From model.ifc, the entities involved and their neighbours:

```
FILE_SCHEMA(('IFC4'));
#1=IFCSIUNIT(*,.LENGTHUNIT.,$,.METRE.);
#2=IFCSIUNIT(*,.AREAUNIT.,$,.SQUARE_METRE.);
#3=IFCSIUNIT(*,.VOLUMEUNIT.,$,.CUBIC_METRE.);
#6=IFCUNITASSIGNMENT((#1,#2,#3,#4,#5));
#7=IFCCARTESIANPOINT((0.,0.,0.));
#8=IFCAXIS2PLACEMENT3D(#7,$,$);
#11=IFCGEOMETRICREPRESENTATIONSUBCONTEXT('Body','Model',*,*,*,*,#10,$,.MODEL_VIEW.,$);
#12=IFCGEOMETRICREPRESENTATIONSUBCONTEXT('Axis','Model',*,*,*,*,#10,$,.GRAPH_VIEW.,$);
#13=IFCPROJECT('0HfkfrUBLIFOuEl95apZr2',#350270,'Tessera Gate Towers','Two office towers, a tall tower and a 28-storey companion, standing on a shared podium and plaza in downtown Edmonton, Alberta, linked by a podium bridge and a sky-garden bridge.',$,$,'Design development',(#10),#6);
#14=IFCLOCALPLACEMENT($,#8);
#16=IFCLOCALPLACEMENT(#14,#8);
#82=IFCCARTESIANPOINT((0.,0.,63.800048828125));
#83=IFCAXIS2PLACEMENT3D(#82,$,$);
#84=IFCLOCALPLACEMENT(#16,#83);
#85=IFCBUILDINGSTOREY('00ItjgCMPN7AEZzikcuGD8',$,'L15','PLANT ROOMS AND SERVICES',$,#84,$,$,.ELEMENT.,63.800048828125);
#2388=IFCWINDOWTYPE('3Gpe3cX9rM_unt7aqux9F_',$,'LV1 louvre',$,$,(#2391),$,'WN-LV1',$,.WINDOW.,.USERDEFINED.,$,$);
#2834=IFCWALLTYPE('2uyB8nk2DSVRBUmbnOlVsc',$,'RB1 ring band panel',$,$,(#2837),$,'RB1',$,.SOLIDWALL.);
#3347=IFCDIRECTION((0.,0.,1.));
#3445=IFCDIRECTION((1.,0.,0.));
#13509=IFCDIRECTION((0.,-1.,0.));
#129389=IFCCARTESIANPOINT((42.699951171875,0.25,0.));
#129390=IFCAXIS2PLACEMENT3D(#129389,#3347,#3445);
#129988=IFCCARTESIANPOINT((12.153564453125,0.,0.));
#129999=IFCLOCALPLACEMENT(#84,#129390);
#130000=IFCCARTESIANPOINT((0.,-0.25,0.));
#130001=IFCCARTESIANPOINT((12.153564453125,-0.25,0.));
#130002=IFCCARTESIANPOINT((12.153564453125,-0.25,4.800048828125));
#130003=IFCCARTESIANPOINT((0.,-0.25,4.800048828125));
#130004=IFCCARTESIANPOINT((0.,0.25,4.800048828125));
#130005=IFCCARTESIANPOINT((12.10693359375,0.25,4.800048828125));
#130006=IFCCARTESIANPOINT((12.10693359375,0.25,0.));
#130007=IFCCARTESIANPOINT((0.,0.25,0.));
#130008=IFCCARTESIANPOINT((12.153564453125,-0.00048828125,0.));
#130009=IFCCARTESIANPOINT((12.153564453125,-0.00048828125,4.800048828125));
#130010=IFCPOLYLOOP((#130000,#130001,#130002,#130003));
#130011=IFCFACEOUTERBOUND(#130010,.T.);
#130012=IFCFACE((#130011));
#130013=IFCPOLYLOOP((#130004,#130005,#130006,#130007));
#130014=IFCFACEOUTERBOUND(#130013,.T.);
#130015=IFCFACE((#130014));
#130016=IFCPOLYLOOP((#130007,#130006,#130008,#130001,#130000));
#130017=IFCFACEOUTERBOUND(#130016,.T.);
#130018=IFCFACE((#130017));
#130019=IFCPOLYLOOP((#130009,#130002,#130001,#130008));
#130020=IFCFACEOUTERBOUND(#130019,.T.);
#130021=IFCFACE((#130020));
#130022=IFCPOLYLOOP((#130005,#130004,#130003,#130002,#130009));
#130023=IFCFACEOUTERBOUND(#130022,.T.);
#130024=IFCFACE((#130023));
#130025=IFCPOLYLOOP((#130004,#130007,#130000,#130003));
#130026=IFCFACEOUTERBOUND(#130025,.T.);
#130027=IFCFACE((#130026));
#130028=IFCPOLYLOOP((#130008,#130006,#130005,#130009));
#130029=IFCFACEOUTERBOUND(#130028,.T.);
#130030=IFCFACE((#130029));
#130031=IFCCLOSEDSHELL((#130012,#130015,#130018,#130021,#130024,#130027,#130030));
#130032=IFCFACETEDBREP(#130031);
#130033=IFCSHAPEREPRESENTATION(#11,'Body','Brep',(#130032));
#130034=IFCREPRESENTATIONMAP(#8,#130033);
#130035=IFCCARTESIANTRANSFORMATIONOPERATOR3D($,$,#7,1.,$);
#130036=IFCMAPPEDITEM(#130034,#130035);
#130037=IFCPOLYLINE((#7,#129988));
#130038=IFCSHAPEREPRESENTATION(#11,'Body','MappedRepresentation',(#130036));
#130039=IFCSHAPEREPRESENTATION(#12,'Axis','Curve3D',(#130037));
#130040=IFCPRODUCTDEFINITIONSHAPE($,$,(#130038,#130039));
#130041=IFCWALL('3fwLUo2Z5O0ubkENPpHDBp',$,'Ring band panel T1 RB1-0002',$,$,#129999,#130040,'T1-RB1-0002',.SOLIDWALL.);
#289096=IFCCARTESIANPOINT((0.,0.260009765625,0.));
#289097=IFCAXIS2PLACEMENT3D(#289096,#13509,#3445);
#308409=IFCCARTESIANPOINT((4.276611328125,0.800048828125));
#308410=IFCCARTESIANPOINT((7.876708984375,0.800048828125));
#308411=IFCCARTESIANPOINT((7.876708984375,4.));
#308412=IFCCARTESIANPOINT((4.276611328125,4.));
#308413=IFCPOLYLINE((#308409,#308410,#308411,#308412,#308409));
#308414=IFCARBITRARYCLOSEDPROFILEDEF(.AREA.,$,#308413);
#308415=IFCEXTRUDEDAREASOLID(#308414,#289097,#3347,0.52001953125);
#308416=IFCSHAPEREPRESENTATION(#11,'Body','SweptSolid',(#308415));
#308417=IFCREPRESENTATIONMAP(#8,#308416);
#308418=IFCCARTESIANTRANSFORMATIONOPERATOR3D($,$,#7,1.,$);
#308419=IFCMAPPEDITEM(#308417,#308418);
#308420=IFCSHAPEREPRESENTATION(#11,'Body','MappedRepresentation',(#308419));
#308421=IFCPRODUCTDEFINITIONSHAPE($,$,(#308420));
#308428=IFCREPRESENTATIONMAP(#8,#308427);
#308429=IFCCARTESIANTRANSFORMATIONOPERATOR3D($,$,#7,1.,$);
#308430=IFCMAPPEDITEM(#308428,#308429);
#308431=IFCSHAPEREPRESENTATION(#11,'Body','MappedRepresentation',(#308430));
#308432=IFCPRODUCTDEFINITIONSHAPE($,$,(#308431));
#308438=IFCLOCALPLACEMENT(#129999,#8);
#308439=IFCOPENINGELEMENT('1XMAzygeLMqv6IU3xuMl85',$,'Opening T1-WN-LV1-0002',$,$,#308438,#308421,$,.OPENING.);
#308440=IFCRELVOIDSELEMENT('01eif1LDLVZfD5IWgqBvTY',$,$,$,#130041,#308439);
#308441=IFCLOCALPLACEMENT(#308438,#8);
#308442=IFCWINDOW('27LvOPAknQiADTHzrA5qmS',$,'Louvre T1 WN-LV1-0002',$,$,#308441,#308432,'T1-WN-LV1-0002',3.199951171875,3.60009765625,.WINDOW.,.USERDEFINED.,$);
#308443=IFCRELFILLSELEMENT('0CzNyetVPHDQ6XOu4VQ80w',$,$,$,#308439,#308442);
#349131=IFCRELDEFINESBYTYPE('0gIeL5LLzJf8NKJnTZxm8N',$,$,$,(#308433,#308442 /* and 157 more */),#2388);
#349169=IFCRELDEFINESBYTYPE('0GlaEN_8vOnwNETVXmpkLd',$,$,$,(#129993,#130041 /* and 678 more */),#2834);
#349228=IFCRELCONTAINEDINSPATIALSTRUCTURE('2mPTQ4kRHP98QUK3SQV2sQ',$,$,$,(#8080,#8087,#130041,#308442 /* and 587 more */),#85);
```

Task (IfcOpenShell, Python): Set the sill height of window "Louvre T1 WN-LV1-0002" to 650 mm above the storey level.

```python
import numpy as np
import ifcopenshell
import ifcopenshell.api.geometry
import ifcopenshell.geom
import ifcopenshell.util.element
import ifcopenshell.util.placement
import ifcopenshell.util.shape
import ifcopenshell.util.unit

model = ifcopenshell.open("model.ifc")
unit_scale = ifcopenshell.util.unit.calculate_unit_scale(model)

window = model.by_guid("27LvOPAknQiADTHzrA5qmS")
opening = window.FillsVoids[0].RelatingOpeningElement
storey = ifcopenshell.util.element.get_container(window, ifc_class="IfcBuildingStorey")
level = ifcopenshell.util.placement.get_local_placement(storey.ObjectPlacement)[2, 3]

# The opening's origin need not be at the sill, so measure its lowest point.
shape = ifcopenshell.geom.create_shape(ifcopenshell.geom.settings(), opening)
bottom = ifcopenshell.util.shape.get_shape_bottom_elevation(shape, shape.geometry) / unit_scale
dz = level + 0.65 / unit_scale - bottom

shift = np.array([0.0, 0.0, dz])
# The window is placed relative to its opening, so it follows when the opening moves.
matrix = ifcopenshell.util.placement.get_local_placement(opening.ObjectPlacement)
matrix[:3, 3] += shift
ifcopenshell.api.geometry.edit_object_placement(
    model, product=opening, matrix=matrix, is_si=False, should_transform_children=True
)

print(f"moved by {dz * unit_scale:+.3f} m")

model.write("model_edited.ifc")
```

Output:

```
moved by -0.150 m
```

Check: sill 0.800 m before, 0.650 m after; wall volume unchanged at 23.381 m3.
